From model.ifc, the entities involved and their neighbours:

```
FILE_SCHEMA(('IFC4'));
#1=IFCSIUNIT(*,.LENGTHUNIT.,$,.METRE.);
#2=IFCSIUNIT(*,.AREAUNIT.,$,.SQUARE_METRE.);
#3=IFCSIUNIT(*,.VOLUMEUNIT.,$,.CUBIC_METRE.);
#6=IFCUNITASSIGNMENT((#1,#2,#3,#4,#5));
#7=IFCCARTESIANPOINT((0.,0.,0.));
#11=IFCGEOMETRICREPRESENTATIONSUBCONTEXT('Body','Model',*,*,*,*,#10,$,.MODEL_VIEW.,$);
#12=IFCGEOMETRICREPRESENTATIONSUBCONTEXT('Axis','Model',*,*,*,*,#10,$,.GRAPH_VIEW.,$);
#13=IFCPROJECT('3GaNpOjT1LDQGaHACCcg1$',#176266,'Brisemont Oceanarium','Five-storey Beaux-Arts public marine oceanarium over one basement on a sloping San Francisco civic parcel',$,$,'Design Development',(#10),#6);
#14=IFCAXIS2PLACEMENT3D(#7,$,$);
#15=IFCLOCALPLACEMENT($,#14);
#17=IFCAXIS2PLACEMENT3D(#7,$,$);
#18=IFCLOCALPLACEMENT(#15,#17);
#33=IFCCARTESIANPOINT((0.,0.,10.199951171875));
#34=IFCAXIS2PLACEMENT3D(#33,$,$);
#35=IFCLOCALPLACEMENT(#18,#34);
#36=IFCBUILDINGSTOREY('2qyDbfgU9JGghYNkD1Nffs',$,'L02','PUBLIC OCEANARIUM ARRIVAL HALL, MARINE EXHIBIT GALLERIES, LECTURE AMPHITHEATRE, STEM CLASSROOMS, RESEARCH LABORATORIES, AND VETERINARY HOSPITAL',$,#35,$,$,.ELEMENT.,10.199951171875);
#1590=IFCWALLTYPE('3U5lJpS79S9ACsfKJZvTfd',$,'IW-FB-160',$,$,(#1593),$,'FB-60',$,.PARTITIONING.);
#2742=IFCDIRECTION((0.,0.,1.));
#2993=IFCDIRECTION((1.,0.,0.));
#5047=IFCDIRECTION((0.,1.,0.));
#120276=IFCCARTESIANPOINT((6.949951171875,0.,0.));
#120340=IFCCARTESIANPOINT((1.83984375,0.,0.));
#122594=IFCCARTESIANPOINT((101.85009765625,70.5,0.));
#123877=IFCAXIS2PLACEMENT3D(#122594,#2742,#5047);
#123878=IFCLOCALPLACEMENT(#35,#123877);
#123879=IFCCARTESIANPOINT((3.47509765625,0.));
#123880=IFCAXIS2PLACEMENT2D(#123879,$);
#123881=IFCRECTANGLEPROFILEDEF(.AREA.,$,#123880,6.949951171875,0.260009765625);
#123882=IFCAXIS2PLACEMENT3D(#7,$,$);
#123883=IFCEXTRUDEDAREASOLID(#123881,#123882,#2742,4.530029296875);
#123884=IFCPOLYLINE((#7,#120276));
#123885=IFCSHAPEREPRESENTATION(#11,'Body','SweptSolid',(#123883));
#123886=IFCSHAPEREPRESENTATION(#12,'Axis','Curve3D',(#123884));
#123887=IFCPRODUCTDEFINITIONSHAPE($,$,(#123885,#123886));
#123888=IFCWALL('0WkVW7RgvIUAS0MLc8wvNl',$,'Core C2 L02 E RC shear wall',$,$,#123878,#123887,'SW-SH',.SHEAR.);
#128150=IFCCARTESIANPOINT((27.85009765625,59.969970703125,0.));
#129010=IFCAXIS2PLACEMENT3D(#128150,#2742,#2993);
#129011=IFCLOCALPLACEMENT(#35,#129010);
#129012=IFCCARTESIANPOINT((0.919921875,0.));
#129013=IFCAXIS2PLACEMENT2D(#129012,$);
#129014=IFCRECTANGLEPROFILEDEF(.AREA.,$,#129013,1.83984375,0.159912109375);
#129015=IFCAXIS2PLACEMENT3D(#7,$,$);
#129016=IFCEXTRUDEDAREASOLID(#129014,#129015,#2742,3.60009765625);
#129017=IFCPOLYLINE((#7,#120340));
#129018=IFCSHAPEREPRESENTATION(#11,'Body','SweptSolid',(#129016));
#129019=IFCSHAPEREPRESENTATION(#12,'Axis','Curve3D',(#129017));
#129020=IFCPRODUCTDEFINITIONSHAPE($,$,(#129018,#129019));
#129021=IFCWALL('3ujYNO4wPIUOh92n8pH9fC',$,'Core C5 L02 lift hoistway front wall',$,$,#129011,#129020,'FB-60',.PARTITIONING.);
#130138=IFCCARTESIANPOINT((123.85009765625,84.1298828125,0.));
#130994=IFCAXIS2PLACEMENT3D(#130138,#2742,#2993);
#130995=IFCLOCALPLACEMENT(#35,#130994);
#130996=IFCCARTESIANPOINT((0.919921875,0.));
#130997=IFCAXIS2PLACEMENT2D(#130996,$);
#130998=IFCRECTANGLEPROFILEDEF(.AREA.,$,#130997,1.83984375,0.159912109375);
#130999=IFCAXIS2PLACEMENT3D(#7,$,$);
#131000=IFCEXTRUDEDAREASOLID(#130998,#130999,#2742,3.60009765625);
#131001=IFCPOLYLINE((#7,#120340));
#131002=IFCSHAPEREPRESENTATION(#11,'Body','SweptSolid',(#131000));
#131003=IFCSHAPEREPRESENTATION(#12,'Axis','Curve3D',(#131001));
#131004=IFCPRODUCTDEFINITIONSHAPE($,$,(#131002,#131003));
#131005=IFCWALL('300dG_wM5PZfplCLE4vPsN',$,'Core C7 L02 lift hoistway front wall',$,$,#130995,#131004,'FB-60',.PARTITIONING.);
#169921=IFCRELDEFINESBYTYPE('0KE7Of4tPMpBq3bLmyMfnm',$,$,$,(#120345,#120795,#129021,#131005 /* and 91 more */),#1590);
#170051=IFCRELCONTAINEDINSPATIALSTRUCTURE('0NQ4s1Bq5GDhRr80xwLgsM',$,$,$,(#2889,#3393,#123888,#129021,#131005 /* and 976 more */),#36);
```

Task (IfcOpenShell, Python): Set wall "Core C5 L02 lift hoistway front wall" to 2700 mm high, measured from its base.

```python
import ifcopenshell
import ifcopenshell.geom
import ifcopenshell.util.representation
import ifcopenshell.util.shape

model = ifcopenshell.open("model.ifc")
settings = ifcopenshell.geom.settings()


def volume(element):
    """Net volume in cubic metres, openings subtracted."""
    shape = ifcopenshell.geom.create_shape(settings, element)
    return ifcopenshell.util.shape.get_volume(shape.geometry)


wall = model.by_guid("3ujYNO4wPIUOh92n8pH9fC")
before = volume(wall)

body = ifcopenshell.util.representation.get_representation(wall, "Model", "Body")
solid = body.Items[0]
old_height = solid.Depth
solid.Depth = 2.7
after = volume(wall)

print(f"height {old_height:g} -> {solid.Depth:g}, volume {before:.3f} -> {after:.3f} m3")

model.write("model_rev.ifc")
```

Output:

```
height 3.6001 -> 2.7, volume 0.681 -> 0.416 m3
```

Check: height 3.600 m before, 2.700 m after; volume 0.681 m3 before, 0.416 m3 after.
